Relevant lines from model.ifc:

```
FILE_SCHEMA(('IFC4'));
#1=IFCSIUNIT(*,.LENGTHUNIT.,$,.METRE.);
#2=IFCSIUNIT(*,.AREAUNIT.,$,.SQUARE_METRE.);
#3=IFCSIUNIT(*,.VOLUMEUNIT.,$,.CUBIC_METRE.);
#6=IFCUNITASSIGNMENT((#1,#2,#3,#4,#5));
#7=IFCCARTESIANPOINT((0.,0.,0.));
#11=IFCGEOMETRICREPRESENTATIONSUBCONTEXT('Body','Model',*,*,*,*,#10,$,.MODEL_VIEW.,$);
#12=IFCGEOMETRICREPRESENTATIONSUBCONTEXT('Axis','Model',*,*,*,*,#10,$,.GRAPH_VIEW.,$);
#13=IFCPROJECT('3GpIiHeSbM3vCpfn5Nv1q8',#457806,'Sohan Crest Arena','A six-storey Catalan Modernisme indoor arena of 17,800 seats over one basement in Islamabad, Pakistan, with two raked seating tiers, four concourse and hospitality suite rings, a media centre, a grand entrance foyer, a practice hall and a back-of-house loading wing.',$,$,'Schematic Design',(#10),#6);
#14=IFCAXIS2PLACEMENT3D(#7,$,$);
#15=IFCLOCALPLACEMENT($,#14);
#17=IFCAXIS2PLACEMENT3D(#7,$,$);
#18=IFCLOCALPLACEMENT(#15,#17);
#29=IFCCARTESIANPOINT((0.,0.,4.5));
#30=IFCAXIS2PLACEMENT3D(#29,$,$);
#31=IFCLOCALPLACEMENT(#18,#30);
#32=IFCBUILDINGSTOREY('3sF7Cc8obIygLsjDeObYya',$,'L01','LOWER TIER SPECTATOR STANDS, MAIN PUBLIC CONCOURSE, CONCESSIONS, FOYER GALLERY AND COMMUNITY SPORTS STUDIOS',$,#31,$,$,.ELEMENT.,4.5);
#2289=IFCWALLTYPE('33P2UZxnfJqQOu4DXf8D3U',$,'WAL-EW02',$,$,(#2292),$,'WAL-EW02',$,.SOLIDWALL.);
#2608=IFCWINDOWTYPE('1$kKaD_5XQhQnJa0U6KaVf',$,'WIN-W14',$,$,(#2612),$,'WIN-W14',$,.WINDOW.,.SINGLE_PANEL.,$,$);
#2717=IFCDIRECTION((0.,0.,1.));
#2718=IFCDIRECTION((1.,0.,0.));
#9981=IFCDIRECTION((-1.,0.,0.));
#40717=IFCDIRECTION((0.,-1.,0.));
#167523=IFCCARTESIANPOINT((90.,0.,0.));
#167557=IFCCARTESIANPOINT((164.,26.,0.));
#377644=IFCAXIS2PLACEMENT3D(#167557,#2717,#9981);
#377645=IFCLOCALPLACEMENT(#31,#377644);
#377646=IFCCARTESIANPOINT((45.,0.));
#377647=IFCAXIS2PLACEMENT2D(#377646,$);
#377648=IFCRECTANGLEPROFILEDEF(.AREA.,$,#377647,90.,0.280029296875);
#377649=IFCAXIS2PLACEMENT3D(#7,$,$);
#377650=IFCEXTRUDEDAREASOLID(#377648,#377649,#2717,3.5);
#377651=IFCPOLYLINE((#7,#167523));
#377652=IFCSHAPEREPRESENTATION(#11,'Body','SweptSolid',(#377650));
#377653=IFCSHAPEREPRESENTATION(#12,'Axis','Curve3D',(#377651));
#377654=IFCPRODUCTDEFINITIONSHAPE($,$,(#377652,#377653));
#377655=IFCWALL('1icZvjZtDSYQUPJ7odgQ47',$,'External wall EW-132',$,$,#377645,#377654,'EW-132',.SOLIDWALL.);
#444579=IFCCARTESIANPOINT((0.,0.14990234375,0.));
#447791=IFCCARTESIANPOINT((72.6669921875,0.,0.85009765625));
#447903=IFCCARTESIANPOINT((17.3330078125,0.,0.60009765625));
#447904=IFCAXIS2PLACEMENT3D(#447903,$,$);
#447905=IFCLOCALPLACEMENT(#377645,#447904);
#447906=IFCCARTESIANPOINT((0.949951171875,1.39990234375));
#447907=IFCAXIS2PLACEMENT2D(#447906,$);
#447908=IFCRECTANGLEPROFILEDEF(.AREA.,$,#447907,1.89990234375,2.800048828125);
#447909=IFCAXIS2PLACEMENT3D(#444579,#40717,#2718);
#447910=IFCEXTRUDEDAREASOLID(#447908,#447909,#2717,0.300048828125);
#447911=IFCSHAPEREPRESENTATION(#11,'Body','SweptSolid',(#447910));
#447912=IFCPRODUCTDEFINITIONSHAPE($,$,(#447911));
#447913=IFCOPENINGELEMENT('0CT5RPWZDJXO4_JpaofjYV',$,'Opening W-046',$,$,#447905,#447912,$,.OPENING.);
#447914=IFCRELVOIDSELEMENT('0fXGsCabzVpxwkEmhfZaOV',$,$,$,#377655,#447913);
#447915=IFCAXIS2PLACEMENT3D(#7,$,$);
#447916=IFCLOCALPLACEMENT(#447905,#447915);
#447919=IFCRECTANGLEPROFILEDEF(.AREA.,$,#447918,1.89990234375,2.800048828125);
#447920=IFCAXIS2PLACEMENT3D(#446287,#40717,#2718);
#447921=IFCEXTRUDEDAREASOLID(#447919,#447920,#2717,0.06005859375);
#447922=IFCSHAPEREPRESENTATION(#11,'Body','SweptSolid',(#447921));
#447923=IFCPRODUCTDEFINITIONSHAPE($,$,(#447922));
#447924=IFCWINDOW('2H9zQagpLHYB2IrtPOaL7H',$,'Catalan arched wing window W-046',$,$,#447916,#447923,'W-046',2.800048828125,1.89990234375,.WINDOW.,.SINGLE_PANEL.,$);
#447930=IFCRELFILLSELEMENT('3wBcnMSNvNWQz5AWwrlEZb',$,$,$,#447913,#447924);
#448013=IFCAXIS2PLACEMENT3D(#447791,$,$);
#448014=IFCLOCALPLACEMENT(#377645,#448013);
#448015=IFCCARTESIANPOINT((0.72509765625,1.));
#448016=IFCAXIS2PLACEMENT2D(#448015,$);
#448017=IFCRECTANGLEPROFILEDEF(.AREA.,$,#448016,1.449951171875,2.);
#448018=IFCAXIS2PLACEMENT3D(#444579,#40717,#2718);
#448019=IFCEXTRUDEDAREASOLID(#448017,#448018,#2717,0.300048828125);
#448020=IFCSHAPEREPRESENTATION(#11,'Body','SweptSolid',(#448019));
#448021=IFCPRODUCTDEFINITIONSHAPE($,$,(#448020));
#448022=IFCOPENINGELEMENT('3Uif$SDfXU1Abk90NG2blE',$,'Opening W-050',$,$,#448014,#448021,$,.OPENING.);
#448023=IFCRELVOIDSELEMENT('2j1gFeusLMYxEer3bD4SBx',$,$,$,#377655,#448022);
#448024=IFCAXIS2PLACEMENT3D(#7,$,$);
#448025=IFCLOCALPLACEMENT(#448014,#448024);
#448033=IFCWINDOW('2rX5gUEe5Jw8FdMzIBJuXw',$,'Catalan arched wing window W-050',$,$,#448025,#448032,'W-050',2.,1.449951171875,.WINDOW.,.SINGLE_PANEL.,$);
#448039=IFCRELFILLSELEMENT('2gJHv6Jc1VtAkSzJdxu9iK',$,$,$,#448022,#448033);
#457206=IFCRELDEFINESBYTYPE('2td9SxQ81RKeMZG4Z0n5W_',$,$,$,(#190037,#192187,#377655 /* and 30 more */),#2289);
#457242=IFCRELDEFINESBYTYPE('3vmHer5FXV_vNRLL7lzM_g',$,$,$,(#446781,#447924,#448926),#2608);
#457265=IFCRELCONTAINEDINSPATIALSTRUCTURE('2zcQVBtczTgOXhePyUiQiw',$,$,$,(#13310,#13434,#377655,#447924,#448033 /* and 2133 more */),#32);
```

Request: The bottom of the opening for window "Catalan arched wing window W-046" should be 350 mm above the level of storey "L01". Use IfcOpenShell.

```python
import numpy as np
import ifcopenshell
import ifcopenshell.api.geometry
import ifcopenshell.geom
import ifcopenshell.util.element
import ifcopenshell.util.placement
import ifcopenshell.util.shape
import ifcopenshell.util.unit

model = ifcopenshell.open("model.ifc")
unit_scale = ifcopenshell.util.unit.calculate_unit_scale(model)

window = model.by_guid("2H9zQagpLHYB2IrtPOaL7H")
opening = window.FillsVoids[0].RelatingOpeningElement
storey = ifcopenshell.util.element.get_container(window, ifc_class="IfcBuildingStorey")
level = ifcopenshell.util.placement.get_local_placement(storey.ObjectPlacement)[2, 3]

# The opening's origin need not be at the sill, so measure its lowest point.
shape = ifcopenshell.geom.create_shape(ifcopenshell.geom.settings(), opening)
bottom = ifcopenshell.util.shape.get_shape_bottom_elevation(shape, shape.geometry) / unit_scale
dz = level + 0.35 / unit_scale - bottom

shift = np.array([0.0, 0.0, dz])
# The window is placed relative to its opening, so it follows when the opening moves.
matrix = ifcopenshell.util.placement.get_local_placement(opening.ObjectPlacement)
matrix[:3, 3] += shift
ifcopenshell.api.geometry.edit_object_placement(
    model, product=opening, matrix=matrix, is_si=False, should_transform_children=True
)

print(f"moved by {dz * unit_scale:+.3f} m")

model.write("model_edited.ifc")
```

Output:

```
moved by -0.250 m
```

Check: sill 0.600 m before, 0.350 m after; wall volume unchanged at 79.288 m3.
